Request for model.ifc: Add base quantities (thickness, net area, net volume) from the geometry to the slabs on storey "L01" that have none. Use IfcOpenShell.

First a look at what the model holds.

```python
import ifcopenshell
import ifcopenshell.util.element
import ifcopenshell.util.unit

model = ifcopenshell.open("model.ifc")
print(model.schema)
for unit_type in ("LENGTHUNIT", "AREAUNIT", "VOLUMEUNIT"):
    print(unit_type, ifcopenshell.util.unit.calculate_unit_scale(model, unit_type))
storey = next(s for s in model.by_type("IfcBuildingStorey") if s.Name == "L01")
slabs = [e for e in ifcopenshell.util.element.get_decomposition(storey) if e.is_a("IfcSlab")]
for e in sorted(slabs, key=lambda e: e.id()):
    print(e.id(), e.is_a(), e.Name, list(ifcopenshell.util.element.get_psets(e, qtos_only=True)), sep=" | ")
```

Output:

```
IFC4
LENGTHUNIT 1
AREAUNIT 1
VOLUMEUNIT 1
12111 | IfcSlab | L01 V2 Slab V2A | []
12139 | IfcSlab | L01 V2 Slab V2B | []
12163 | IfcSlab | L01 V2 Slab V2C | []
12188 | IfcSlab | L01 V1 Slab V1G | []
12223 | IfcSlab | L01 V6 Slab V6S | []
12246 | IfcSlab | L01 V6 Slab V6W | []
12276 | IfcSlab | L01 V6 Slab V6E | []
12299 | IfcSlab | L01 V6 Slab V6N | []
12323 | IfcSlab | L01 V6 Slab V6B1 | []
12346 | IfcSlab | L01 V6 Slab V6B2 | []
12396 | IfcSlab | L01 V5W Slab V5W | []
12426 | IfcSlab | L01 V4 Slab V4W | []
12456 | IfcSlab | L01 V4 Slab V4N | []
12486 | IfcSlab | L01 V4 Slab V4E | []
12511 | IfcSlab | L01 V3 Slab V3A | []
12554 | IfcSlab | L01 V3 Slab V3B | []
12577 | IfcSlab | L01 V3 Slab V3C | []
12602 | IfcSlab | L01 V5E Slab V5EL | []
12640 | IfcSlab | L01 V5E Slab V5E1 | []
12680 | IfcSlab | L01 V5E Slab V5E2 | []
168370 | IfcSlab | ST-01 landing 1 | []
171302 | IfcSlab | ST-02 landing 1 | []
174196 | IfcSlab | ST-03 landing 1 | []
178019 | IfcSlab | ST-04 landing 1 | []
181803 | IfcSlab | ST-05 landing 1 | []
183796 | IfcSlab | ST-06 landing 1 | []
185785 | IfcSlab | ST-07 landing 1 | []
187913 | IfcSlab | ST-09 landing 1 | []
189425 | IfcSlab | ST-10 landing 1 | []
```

```python
import ifcopenshell
import ifcopenshell.api.pset
import ifcopenshell.geom
import ifcopenshell.util.element
import ifcopenshell.util.shape
import ifcopenshell.util.unit

model = ifcopenshell.open("model.ifc")
unit_scale = ifcopenshell.util.unit.calculate_unit_scale(model)
area_scale = ifcopenshell.util.unit.calculate_unit_scale(model, "AREAUNIT")
volume_scale = ifcopenshell.util.unit.calculate_unit_scale(model, "VOLUMEUNIT")
settings = ifcopenshell.geom.settings()

storey = next(s for s in model.by_type("IfcBuildingStorey") if s.Name == "L01")
slabs = [e for e in ifcopenshell.util.element.get_decomposition(storey) if e.is_a("IfcSlab")]

for e in sorted(slabs, key=lambda e: e.id()):
    if ifcopenshell.util.element.get_psets(e, qtos_only=True, should_inherit=False):
        continue
    # Geometry comes back in metres, in the element's own axes.
    shape = ifcopenshell.geom.create_shape(settings, e)
    values = {
        "Width": ifcopenshell.util.shape.get_z(shape.geometry) / unit_scale,
        "NetArea": ifcopenshell.util.shape.get_footprint_area(shape.geometry) / area_scale,
        "NetVolume": ifcopenshell.util.shape.get_volume(shape.geometry) / volume_scale,
    }
    qto = ifcopenshell.api.pset.add_qto(model, product=e, name="Qto_SlabBaseQuantities")
    ifcopenshell.api.pset.edit_qto(model, qto=qto, properties=values)
    print(e.id(), {k: round(v, 3) for k, v in values.items()})

model.write("model_updated.ifc")
```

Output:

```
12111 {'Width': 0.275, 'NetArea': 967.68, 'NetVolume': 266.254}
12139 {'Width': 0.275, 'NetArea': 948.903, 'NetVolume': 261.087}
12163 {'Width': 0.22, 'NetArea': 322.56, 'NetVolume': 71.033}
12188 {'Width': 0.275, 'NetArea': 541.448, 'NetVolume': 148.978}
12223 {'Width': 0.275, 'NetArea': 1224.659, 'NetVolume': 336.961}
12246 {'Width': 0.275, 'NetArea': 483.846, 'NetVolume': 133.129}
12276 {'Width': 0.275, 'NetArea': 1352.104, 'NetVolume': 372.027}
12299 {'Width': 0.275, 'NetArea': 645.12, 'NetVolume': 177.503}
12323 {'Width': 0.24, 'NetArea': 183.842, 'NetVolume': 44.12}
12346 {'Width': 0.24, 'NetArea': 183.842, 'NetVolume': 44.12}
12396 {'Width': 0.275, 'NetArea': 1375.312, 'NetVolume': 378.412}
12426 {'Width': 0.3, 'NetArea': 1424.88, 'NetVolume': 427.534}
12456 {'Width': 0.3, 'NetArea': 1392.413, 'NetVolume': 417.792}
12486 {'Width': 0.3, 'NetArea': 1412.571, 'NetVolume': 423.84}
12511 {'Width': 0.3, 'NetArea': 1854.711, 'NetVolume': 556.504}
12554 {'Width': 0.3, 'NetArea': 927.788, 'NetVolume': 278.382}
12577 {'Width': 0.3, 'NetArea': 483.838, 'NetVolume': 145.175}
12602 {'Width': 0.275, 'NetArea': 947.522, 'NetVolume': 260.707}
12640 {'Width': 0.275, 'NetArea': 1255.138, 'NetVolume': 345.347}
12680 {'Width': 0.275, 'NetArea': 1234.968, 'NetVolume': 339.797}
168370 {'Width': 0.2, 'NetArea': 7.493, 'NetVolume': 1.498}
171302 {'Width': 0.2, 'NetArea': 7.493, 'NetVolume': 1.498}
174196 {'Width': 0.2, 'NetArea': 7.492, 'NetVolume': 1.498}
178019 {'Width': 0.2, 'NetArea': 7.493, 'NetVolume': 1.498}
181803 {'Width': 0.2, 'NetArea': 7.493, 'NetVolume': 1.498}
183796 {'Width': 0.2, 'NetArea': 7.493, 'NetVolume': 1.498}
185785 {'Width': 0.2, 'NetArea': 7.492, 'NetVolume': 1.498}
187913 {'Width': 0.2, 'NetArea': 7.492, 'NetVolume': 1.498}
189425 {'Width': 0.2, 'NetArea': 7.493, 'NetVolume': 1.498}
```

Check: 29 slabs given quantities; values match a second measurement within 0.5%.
